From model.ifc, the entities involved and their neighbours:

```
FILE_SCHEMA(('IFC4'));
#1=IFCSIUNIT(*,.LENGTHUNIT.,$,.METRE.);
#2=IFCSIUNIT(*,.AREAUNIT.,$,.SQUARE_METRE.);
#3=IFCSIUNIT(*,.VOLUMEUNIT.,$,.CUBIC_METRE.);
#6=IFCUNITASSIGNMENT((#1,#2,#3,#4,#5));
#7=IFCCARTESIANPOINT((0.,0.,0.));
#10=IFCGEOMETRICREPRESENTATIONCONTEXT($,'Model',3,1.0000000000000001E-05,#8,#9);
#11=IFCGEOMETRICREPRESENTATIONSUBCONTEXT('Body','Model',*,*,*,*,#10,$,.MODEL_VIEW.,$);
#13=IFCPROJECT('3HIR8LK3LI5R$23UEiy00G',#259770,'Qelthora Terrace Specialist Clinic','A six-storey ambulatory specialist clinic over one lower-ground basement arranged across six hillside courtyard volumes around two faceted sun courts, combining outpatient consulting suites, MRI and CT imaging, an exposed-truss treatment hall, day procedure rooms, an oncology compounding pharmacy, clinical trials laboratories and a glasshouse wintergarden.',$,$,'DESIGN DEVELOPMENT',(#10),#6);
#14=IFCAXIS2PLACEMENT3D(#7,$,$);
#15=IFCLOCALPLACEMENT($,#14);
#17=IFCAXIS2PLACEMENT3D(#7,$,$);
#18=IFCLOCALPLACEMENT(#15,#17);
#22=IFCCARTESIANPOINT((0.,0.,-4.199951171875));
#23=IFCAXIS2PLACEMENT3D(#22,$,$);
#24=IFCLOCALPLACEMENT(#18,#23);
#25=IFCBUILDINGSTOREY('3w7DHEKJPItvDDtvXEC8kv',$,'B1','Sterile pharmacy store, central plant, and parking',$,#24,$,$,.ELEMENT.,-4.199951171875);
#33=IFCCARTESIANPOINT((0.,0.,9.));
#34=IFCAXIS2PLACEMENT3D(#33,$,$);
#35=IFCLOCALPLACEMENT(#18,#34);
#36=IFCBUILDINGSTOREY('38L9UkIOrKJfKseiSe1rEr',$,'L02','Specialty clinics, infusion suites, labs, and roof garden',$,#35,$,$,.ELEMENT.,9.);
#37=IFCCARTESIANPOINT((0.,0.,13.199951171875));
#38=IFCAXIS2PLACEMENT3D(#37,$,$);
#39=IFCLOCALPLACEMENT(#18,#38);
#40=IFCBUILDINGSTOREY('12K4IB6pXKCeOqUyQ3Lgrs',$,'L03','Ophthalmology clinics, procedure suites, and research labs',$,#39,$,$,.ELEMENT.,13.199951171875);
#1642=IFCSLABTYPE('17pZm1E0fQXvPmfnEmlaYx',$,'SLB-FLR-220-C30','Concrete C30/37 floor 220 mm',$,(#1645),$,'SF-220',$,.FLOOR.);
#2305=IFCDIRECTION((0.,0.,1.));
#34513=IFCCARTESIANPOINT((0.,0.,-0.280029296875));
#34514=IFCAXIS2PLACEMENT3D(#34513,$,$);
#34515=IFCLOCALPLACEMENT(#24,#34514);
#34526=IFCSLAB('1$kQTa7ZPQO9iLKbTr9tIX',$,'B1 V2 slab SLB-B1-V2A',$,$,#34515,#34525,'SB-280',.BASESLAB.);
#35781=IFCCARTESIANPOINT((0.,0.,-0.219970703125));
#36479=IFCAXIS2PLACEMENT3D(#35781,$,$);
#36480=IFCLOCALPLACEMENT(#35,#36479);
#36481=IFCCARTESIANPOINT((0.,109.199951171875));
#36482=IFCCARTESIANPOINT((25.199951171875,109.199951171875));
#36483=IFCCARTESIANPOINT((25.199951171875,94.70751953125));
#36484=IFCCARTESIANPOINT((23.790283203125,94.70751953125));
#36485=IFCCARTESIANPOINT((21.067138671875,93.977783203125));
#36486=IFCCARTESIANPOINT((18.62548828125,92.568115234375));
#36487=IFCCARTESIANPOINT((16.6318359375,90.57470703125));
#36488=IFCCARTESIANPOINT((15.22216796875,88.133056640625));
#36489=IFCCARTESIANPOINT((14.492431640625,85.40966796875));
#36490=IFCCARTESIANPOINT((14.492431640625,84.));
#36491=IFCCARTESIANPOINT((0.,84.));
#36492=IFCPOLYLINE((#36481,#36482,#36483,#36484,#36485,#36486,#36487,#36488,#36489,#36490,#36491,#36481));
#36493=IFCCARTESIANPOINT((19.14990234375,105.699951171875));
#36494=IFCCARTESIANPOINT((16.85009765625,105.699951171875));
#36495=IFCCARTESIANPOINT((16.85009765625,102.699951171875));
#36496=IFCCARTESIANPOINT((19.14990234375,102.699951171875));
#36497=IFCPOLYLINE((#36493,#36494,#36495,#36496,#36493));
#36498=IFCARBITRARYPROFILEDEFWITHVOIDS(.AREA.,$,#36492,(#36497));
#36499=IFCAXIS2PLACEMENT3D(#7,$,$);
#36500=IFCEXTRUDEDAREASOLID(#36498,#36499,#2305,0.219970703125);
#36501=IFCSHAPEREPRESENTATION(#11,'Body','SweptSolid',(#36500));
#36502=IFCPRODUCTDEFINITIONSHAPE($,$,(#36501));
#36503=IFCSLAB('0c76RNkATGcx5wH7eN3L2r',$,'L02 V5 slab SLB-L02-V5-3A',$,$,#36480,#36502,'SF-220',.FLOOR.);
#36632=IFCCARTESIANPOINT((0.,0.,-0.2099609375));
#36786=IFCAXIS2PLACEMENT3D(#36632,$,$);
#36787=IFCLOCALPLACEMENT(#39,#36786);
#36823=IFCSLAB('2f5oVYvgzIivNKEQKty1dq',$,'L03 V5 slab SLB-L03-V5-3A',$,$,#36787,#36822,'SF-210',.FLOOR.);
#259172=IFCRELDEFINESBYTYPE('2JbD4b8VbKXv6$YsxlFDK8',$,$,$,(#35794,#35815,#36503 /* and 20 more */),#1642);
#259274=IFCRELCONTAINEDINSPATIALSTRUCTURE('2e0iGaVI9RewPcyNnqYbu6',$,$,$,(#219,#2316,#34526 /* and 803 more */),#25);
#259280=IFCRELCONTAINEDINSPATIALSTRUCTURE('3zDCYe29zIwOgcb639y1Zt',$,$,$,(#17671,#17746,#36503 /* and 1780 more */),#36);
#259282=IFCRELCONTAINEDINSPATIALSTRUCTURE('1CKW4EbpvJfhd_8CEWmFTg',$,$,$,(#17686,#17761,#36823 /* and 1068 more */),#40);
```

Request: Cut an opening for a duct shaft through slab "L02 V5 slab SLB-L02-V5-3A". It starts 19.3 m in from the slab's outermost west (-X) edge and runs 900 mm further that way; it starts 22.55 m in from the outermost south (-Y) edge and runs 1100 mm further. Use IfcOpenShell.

```python
import numpy as np
import ifcopenshell
import ifcopenshell.api.feature
import ifcopenshell.api.geometry
import ifcopenshell.api.root
import ifcopenshell.geom
import ifcopenshell.util.placement
import ifcopenshell.util.representation
import ifcopenshell.util.shape
import ifcopenshell.util.unit

model = ifcopenshell.open("model.ifc")
unit_scale = ifcopenshell.util.unit.calculate_unit_scale(model)
settings = ifcopenshell.geom.settings()


def volume(element):
    """Net volume in cubic metres, openings subtracted."""
    shape = ifcopenshell.geom.create_shape(settings, element)
    return ifcopenshell.util.shape.get_volume(shape.geometry)


slab = model.by_guid("0c76RNkATGcx5wH7eN3L2r")
before = volume(slab)

# Extent in the slab's own axes, in metres. The edges named are its -X and -Y sides.
slab_shape = ifcopenshell.geom.create_shape(settings, slab)
vertices = ifcopenshell.util.shape.get_vertices(slab_shape.geometry)
x_min, y_min, bottom = vertices.min(axis=0)
top = vertices[:, 2].max()

opening = ifcopenshell.api.root.create_entity(model, ifc_class="IfcOpeningElement", name="Duct shaft opening", predefined_type="OPENING")
context = ifcopenshell.util.representation.get_context(model, "Model", "Body", "MODEL_VIEW")
width, depth = 0.9, 1.1
outline = [(0.0, 0.0), (width, 0.0), (width, depth), (0.0, depth), (0.0, 0.0)]
# Overshoot both faces by 50 mm so the cut is clean.
shape = ifcopenshell.api.geometry.add_slab_representation(
    model, context=context, depth=top - bottom + 0.1, polyline=outline
)
ifcopenshell.api.geometry.assign_representation(model, product=opening, representation=shape)

matrix = ifcopenshell.util.placement.get_local_placement(slab.ObjectPlacement)
matrix[:, 3] = matrix @ np.append(np.array([x_min + 19.3, y_min + 22.55, bottom - 0.05]) / unit_scale, 1.0)
ifcopenshell.api.geometry.edit_object_placement(model, product=opening, matrix=matrix, is_si=False)
ifcopenshell.api.feature.add_feature(model, feature=opening, element=slab)

after = volume(slab)

print(f"slab volume {before:.3f} -> {after:.3f} m3")

model.write("model_v2.ifc")
```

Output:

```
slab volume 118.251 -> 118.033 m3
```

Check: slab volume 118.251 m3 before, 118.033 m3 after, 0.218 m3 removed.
